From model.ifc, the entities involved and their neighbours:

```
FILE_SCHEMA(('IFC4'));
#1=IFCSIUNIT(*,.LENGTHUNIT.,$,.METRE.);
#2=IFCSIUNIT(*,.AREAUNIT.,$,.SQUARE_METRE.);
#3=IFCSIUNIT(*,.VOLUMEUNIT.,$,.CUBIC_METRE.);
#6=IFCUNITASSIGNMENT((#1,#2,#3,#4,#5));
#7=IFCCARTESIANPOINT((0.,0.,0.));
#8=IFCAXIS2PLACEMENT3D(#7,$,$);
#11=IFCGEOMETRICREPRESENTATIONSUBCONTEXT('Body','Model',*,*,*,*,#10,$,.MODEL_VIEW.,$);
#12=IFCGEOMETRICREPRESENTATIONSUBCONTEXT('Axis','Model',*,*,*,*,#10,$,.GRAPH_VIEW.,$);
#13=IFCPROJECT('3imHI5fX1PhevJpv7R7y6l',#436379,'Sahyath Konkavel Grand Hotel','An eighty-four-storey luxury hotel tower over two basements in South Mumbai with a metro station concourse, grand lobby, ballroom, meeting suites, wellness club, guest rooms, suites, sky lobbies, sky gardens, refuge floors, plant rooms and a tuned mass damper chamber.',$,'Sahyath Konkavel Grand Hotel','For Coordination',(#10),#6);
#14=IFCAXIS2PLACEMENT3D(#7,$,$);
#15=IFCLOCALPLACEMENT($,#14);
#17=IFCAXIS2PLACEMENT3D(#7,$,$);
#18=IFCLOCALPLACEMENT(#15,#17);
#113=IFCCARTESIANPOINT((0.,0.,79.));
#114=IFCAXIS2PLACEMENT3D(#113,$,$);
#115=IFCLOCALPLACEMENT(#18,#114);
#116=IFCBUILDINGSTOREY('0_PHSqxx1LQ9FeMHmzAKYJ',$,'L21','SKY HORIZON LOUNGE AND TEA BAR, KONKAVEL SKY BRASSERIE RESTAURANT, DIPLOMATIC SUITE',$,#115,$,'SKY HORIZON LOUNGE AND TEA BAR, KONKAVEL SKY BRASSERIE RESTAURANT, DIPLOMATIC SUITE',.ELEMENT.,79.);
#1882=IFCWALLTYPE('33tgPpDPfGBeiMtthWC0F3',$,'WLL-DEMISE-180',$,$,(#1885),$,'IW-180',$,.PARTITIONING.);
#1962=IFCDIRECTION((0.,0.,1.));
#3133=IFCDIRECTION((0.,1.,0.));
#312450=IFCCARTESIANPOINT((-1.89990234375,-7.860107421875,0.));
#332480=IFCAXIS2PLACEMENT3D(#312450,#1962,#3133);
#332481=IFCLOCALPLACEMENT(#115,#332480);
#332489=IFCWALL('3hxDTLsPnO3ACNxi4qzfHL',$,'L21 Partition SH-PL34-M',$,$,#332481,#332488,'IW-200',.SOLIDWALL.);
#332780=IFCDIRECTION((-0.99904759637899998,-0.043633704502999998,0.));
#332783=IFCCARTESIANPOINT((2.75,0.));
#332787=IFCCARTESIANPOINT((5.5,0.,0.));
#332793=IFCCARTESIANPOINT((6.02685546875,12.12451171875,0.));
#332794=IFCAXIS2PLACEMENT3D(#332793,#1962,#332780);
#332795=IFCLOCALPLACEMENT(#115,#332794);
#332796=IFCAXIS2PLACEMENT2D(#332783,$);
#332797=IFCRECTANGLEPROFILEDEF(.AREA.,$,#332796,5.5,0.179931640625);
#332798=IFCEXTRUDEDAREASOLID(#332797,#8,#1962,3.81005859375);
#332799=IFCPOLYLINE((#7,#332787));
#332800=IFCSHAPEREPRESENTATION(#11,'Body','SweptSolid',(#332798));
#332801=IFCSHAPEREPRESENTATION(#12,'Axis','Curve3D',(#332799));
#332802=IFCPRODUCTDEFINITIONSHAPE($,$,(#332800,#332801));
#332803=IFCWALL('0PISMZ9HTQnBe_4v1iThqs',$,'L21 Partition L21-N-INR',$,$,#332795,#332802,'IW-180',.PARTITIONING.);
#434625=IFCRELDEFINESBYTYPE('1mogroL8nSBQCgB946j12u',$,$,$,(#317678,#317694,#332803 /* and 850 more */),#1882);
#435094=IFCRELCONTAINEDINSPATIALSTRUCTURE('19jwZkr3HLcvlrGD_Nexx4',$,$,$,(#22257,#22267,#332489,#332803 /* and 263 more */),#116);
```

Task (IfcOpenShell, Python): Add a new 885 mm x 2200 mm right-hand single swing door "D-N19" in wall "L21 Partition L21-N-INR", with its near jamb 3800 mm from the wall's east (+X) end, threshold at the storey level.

```python
import numpy as np
import ifcopenshell
import ifcopenshell.api.feature
import ifcopenshell.api.geometry
import ifcopenshell.api.root
import ifcopenshell.api.spatial
import ifcopenshell.geom
import ifcopenshell.util.element
import ifcopenshell.util.placement
import ifcopenshell.util.representation
import ifcopenshell.util.shape
import ifcopenshell.util.unit

model = ifcopenshell.open("model.ifc")
unit_scale = ifcopenshell.util.unit.calculate_unit_scale(model)
settings = ifcopenshell.geom.settings()


def volume(element):
    """Net volume in cubic metres, openings subtracted."""
    shape = ifcopenshell.geom.create_shape(settings, element)
    return ifcopenshell.util.shape.get_volume(shape.geometry)


wall = model.by_guid("0PISMZ9HTQnBe_4v1iThqs")
storey = ifcopenshell.util.element.get_container(wall, ifc_class="IfcBuildingStorey")
context = ifcopenshell.util.representation.get_context(model, "Model", "Body", "MODEL_VIEW")
before = volume(wall)

width, height, from_end, sill = 0.885, 2.2, 3.8, 0.0  # metres

# The wall runs along its own X axis, and the end named is its -X end.
wall_shape = ifcopenshell.geom.create_shape(settings, wall)
x, y, z = ifcopenshell.util.shape.get_vertices(wall_shape.geometry).T
start = x.min() + from_end
face, thickness = float(y.min()), float(y.max() - y.min())
wall_matrix = ifcopenshell.util.placement.get_local_placement(wall.ObjectPlacement)
level = ifcopenshell.util.placement.get_local_placement(storey.ObjectPlacement)[2, 3]


def in_wall(x, y):
    """Placement at x, y metres in the wall's axes, at sill height."""
    matrix = wall_matrix.copy()
    matrix[:, 3] = wall_matrix @ np.array([x / unit_scale, y / unit_scale, 0.0, 1.0])
    matrix[2, 3] = level + sill / unit_scale
    return matrix


# Opening: a box that overshoots both wall faces by 50 mm.
opening = ifcopenshell.api.root.create_entity(model, ifc_class="IfcOpeningElement", predefined_type="OPENING")
box = ifcopenshell.api.geometry.add_wall_representation(
    model, context=context, length=width, height=height, thickness=thickness + 0.1
)
ifcopenshell.api.geometry.assign_representation(model, product=opening, representation=box)
ifcopenshell.api.geometry.edit_object_placement(model, product=opening, matrix=in_wall(start, face - 0.05), is_si=False)
ifcopenshell.api.feature.add_feature(model, feature=opening, element=wall)

door = ifcopenshell.api.root.create_entity(model, ifc_class="IfcDoor", name="D-N19", predefined_type="DOOR")
door.OverallWidth, door.OverallHeight = width / unit_scale, height / unit_scale
door.OperationType = "SINGLE_SWING_RIGHT"
body = ifcopenshell.api.geometry.add_door_representation(
    model,
    context=context,
    overall_width=door.OverallWidth,
    overall_height=door.OverallHeight,
    operation_type="SINGLE_SWING_RIGHT",
    lining_properties={"LiningDepth": thickness / unit_scale, "ThresholdDepth": thickness / unit_scale},
)
ifcopenshell.api.geometry.assign_representation(model, product=door, representation=body)
ifcopenshell.api.spatial.assign_container(model, products=[door], relating_structure=storey)
ifcopenshell.api.feature.add_filling(model, opening=opening, element=door)

# The lining spans the wall, so the door starts at the wall face.
ifcopenshell.api.geometry.edit_object_placement(model, product=door, matrix=in_wall(start, face), is_si=False)

after = volume(wall)

print(f"wall volume {before:.3f} -> {after:.3f} m3")

model.write("model_updated.ifc")
```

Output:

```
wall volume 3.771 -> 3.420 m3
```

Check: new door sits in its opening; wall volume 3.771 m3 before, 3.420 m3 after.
